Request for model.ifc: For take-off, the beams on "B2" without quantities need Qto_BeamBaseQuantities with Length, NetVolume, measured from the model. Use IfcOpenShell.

First a look at what the model holds.

```python
import ifcopenshell
import ifcopenshell.util.element
import ifcopenshell.util.unit

model = ifcopenshell.open("model.ifc")
print(model.schema)
for unit_type in ("LENGTHUNIT", "AREAUNIT", "VOLUMEUNIT"):
    print(unit_type, ifcopenshell.util.unit.calculate_unit_scale(model, unit_type))
storey = next(s for s in model.by_type("IfcBuildingStorey") if s.Name == "B2")
beams = [e for e in ifcopenshell.util.element.get_decomposition(storey) if e.is_a("IfcBeam")]
for e in sorted(beams, key=lambda e: e.id()):
    print(e.id(), e.is_a(), e.Name, list(ifcopenshell.util.element.get_psets(e, qtos_only=True)), sep=" | ")
```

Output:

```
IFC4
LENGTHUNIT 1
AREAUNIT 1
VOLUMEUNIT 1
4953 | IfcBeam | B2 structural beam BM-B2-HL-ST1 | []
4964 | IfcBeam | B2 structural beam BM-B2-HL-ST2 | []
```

```python
import ifcopenshell
import ifcopenshell.api.pset
import ifcopenshell.geom
import ifcopenshell.util.element
import ifcopenshell.util.shape
import ifcopenshell.util.unit

model = ifcopenshell.open("model.ifc")
unit_scale = ifcopenshell.util.unit.calculate_unit_scale(model)
volume_scale = ifcopenshell.util.unit.calculate_unit_scale(model, "VOLUMEUNIT")
settings = ifcopenshell.geom.settings()

storey = next(s for s in model.by_type("IfcBuildingStorey") if s.Name == "B2")
beams = [e for e in ifcopenshell.util.element.get_decomposition(storey) if e.is_a("IfcBeam")]

for e in sorted(beams, key=lambda e: e.id()):
    if ifcopenshell.util.element.get_psets(e, qtos_only=True, should_inherit=False):
        continue
    # Geometry comes back in metres, in the element's own axes.
    shape = ifcopenshell.geom.create_shape(settings, e)
    values = {
        "Length": ifcopenshell.util.shape.get_max_xyz(shape.geometry) / unit_scale,
        "NetVolume": ifcopenshell.util.shape.get_volume(shape.geometry) / volume_scale,
    }
    qto = ifcopenshell.api.pset.add_qto(model, product=e, name="Qto_BeamBaseQuantities")
    ifcopenshell.api.pset.edit_qto(model, qto=qto, properties=values)
    print(e.id(), {k: round(v, 3) for k, v in values.items()})

model.write("model_edited.ifc")
```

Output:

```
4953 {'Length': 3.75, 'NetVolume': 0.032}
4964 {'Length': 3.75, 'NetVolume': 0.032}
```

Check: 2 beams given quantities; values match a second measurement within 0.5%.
